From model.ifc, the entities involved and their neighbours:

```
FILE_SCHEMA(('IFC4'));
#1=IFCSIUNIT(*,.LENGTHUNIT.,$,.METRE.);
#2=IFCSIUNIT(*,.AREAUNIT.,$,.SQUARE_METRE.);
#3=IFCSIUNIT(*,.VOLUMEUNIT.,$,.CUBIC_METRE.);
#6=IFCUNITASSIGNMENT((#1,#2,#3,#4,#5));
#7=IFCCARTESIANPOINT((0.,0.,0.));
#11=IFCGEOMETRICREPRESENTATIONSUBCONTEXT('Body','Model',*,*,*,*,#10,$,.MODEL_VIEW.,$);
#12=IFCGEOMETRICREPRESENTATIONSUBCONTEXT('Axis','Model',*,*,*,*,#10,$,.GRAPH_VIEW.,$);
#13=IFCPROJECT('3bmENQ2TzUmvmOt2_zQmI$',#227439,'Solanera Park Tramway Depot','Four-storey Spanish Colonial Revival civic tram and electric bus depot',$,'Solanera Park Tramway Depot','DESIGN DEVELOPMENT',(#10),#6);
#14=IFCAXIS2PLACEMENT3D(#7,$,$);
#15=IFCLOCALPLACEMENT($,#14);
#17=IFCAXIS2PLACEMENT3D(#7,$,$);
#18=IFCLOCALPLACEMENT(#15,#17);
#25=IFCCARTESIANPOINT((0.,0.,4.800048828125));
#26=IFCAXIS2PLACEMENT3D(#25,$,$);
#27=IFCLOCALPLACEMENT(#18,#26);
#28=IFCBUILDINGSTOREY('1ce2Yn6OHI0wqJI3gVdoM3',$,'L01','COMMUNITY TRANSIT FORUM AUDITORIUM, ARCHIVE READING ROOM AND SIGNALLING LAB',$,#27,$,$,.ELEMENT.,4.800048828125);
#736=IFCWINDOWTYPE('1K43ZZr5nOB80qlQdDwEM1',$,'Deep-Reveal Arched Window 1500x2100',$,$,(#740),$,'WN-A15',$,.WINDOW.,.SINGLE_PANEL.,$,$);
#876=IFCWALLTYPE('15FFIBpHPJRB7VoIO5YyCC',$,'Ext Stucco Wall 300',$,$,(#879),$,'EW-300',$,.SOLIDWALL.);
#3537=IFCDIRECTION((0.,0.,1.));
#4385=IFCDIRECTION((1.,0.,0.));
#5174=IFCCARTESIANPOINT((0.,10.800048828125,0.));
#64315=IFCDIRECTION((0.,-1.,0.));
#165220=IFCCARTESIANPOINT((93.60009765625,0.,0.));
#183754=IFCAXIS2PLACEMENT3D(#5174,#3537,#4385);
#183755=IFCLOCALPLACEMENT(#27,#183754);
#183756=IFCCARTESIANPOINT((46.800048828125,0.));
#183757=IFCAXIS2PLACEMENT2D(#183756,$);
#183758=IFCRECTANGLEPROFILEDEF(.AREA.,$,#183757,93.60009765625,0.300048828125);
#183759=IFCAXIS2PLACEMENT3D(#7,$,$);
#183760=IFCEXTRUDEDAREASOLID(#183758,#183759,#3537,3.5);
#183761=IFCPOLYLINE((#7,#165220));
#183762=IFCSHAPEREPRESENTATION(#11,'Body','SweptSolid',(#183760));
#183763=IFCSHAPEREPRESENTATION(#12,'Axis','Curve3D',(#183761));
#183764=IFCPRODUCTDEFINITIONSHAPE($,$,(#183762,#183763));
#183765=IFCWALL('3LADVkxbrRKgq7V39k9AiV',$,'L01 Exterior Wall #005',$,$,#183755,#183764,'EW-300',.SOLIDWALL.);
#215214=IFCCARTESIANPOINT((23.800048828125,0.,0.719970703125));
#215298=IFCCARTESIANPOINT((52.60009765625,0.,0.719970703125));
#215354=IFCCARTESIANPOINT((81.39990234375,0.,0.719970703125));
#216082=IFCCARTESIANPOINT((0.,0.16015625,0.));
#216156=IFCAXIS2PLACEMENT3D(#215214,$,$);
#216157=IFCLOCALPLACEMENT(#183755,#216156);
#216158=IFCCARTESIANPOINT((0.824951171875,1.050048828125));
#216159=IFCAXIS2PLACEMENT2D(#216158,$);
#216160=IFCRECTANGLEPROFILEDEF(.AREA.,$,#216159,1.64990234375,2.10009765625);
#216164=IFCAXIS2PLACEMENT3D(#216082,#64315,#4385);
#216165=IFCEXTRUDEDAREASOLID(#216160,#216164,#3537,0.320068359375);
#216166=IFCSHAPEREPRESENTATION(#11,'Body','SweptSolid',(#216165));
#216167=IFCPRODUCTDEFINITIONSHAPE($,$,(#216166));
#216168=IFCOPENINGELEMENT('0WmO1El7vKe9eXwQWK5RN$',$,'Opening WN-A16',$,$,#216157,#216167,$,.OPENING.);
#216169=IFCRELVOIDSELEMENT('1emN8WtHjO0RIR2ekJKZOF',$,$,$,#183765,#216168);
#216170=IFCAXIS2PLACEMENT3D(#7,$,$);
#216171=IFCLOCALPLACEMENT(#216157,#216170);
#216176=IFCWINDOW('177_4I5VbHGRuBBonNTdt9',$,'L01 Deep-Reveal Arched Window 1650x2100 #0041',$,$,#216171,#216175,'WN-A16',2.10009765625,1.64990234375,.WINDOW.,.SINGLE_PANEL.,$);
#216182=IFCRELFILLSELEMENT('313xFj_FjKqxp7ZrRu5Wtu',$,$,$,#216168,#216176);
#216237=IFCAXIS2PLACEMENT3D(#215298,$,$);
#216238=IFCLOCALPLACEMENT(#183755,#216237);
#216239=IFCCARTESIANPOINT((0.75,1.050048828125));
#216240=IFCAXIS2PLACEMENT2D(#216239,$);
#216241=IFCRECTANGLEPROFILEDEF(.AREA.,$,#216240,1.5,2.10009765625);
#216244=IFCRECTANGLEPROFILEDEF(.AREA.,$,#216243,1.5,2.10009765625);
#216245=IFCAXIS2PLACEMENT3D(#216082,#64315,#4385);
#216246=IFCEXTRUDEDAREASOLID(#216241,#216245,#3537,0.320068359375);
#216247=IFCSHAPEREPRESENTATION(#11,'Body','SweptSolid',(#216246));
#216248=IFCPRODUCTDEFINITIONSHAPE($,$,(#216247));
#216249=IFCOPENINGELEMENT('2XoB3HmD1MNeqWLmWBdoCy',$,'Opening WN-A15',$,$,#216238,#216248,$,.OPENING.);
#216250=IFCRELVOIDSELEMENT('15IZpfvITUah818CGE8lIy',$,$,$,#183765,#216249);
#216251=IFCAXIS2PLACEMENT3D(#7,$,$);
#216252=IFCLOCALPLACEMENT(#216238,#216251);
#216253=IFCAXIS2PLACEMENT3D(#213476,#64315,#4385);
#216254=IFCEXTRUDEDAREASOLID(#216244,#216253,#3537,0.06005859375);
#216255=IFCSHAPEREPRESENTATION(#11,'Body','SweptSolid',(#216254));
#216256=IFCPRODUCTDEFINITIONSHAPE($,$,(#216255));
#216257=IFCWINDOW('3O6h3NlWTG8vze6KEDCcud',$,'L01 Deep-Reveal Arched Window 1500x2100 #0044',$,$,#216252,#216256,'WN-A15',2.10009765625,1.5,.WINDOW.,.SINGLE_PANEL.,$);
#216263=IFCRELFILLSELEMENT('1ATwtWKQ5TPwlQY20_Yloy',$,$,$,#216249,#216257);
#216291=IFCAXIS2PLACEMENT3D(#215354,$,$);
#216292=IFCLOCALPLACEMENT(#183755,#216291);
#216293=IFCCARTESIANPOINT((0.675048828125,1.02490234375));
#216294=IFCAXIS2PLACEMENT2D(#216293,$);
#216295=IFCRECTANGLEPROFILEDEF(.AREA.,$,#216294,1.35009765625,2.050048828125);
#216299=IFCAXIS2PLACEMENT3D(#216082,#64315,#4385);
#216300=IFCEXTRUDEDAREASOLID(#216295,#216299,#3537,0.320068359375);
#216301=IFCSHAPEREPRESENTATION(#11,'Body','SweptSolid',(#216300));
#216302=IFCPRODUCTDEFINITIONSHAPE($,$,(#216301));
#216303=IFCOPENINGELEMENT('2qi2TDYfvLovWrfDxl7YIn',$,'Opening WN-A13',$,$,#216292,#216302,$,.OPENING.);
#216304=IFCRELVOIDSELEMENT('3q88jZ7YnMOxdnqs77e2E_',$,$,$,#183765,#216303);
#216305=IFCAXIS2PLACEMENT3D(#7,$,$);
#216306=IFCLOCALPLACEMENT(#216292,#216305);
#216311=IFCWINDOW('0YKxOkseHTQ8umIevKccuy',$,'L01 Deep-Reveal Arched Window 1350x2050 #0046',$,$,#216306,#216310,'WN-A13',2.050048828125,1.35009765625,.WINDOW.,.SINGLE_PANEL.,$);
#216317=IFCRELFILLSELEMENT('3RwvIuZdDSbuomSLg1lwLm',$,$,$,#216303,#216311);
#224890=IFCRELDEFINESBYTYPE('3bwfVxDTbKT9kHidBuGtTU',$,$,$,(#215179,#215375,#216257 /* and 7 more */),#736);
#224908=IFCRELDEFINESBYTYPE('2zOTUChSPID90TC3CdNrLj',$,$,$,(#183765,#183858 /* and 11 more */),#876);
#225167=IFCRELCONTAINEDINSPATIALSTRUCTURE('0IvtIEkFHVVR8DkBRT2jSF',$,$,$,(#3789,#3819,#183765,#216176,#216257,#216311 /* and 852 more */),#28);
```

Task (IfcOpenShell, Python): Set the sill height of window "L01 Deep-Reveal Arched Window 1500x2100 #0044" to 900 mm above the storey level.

```python
import numpy as np
import ifcopenshell
import ifcopenshell.api.geometry
import ifcopenshell.geom
import ifcopenshell.util.element
import ifcopenshell.util.placement
import ifcopenshell.util.shape
import ifcopenshell.util.unit

model = ifcopenshell.open("model.ifc")
unit_scale = ifcopenshell.util.unit.calculate_unit_scale(model)

window = model.by_id(216257)
opening = window.FillsVoids[0].RelatingOpeningElement
storey = ifcopenshell.util.element.get_container(window, ifc_class="IfcBuildingStorey")
level = ifcopenshell.util.placement.get_local_placement(storey.ObjectPlacement)[2, 3]

# The opening's origin need not be at the sill, so measure its lowest point.
shape = ifcopenshell.geom.create_shape(ifcopenshell.geom.settings(), opening)
bottom = ifcopenshell.util.shape.get_shape_bottom_elevation(shape, shape.geometry) / unit_scale
dz = level + 0.9 / unit_scale - bottom

shift = np.array([0.0, 0.0, dz])
# The window is placed relative to its opening, so it follows when the opening moves.
matrix = ifcopenshell.util.placement.get_local_placement(opening.ObjectPlacement)
matrix[:3, 3] += shift
ifcopenshell.api.geometry.edit_object_placement(
    model, product=opening, matrix=matrix, is_si=False, should_transform_children=True
)

print(f"moved by {dz * unit_scale:+.3f} m")

model.write("model_updated.ifc")
```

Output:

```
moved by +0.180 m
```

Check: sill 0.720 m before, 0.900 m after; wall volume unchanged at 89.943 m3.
